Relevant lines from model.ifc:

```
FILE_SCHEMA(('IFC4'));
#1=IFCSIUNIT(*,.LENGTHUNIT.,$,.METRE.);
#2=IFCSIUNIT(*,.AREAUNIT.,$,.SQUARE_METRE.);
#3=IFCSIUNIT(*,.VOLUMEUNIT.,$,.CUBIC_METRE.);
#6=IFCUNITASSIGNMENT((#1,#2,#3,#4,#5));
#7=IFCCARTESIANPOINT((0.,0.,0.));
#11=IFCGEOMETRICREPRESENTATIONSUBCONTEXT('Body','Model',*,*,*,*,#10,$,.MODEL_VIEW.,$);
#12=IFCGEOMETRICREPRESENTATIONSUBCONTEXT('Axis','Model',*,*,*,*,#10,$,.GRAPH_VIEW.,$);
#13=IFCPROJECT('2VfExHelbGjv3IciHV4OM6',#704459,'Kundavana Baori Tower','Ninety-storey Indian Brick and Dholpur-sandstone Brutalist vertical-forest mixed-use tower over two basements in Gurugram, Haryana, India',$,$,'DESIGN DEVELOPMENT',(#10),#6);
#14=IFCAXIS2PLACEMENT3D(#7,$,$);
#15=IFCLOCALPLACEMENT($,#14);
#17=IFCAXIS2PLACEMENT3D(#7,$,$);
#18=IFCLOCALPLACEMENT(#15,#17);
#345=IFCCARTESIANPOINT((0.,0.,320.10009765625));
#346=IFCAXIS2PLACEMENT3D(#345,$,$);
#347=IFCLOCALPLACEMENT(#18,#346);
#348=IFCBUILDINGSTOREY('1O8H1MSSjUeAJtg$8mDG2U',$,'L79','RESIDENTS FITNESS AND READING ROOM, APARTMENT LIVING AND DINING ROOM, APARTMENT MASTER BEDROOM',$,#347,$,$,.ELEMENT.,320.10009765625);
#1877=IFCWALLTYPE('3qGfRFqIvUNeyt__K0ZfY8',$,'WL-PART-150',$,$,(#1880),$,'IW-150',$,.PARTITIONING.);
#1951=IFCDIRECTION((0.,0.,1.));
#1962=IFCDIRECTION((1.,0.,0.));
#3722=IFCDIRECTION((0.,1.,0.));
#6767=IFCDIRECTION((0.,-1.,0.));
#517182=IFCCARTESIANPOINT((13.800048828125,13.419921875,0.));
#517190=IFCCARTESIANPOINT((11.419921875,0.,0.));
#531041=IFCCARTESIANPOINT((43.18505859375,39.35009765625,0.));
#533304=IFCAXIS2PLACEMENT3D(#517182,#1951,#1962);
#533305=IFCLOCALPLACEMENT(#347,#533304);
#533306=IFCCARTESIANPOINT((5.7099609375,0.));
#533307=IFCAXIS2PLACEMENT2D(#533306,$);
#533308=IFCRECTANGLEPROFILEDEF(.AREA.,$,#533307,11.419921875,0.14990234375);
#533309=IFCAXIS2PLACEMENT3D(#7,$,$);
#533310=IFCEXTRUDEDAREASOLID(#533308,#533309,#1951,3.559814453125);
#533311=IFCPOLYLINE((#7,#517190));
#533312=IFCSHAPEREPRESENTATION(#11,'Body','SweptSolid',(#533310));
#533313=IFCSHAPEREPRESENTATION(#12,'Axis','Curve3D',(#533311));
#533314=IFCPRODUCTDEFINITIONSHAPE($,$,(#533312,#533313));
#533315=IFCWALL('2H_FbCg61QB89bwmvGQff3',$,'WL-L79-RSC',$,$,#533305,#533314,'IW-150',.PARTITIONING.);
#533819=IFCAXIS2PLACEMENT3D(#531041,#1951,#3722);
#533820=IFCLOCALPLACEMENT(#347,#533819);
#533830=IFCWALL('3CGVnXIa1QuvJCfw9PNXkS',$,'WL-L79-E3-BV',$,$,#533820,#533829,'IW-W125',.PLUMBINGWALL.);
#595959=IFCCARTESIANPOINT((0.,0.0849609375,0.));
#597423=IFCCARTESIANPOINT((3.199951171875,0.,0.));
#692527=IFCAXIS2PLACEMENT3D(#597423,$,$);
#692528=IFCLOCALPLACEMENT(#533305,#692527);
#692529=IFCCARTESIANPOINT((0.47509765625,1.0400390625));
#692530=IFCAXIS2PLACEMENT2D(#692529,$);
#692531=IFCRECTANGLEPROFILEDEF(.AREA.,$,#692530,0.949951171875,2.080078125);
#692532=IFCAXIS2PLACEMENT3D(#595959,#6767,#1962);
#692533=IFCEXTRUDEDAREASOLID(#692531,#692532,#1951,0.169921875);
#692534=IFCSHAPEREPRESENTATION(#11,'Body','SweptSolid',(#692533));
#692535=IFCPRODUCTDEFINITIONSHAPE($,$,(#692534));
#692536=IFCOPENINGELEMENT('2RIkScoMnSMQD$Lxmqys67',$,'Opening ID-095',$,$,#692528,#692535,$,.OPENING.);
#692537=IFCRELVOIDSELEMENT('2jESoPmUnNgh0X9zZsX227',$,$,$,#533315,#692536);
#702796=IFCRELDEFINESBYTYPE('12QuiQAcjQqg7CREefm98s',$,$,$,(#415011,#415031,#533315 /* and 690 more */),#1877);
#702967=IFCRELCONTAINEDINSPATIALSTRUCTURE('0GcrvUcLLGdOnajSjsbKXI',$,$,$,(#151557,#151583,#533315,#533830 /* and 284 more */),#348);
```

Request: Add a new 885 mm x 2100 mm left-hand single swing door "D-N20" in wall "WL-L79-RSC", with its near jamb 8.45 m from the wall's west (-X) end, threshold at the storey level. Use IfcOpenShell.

```python
import numpy as np
import ifcopenshell
import ifcopenshell.api.feature
import ifcopenshell.api.geometry
import ifcopenshell.api.root
import ifcopenshell.api.spatial
import ifcopenshell.geom
import ifcopenshell.util.element
import ifcopenshell.util.placement
import ifcopenshell.util.representation
import ifcopenshell.util.shape
import ifcopenshell.util.unit

model = ifcopenshell.open("model.ifc")
unit_scale = ifcopenshell.util.unit.calculate_unit_scale(model)
settings = ifcopenshell.geom.settings()


def volume(element):
    """Net volume in cubic metres, openings subtracted."""
    shape = ifcopenshell.geom.create_shape(settings, element)
    return ifcopenshell.util.shape.get_volume(shape.geometry)


wall = model.by_guid("2H_FbCg61QB89bwmvGQff3")
storey = ifcopenshell.util.element.get_container(wall, ifc_class="IfcBuildingStorey")
context = ifcopenshell.util.representation.get_context(model, "Model", "Body", "MODEL_VIEW")
before = volume(wall)

width, height, from_end, sill = 0.885, 2.1, 8.45, 0.0  # metres

# The wall runs along its own X axis, and the end named is its -X end.
wall_shape = ifcopenshell.geom.create_shape(settings, wall)
x, y, z = ifcopenshell.util.shape.get_vertices(wall_shape.geometry).T
start = x.min() + from_end
face, thickness = float(y.min()), float(y.max() - y.min())
wall_matrix = ifcopenshell.util.placement.get_local_placement(wall.ObjectPlacement)
level = ifcopenshell.util.placement.get_local_placement(storey.ObjectPlacement)[2, 3]


def in_wall(x, y):
    """Placement at x, y metres in the wall's axes, at sill height."""
    matrix = wall_matrix.copy()
    matrix[:, 3] = wall_matrix @ np.array([x / unit_scale, y / unit_scale, 0.0, 1.0])
    matrix[2, 3] = level + sill / unit_scale
    return matrix


# Opening: a box that overshoots both wall faces by 50 mm.
opening = ifcopenshell.api.root.create_entity(model, ifc_class="IfcOpeningElement", predefined_type="OPENING")
box = ifcopenshell.api.geometry.add_wall_representation(
    model, context=context, length=width, height=height, thickness=thickness + 0.1
)
ifcopenshell.api.geometry.assign_representation(model, product=opening, representation=box)
ifcopenshell.api.geometry.edit_object_placement(model, product=opening, matrix=in_wall(start, face - 0.05), is_si=False)
ifcopenshell.api.feature.add_feature(model, feature=opening, element=wall)

door = ifcopenshell.api.root.create_entity(model, ifc_class="IfcDoor", name="D-N20", predefined_type="DOOR")
door.OverallWidth, door.OverallHeight = width / unit_scale, height / unit_scale
door.OperationType = "SINGLE_SWING_LEFT"
body = ifcopenshell.api.geometry.add_door_representation(
    model,
    context=context,
    overall_width=door.OverallWidth,
    overall_height=door.OverallHeight,
    operation_type="SINGLE_SWING_LEFT",
    lining_properties={"LiningDepth": thickness / unit_scale, "ThresholdDepth": thickness / unit_scale},
)
ifcopenshell.api.geometry.assign_representation(model, product=door, representation=body)
ifcopenshell.api.spatial.assign_container(model, products=[door], relating_structure=storey)
ifcopenshell.api.feature.add_filling(model, opening=opening, element=door)

# The lining spans the wall, so the door starts at the wall face.
ifcopenshell.api.geometry.edit_object_placement(model, product=door, matrix=in_wall(start, face), is_si=False)

after = volume(wall)

print(f"wall volume {before:.3f} -> {after:.3f} m3")

model.write("model_rev.ifc")
```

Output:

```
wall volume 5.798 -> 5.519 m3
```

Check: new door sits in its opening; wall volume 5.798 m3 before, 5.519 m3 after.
